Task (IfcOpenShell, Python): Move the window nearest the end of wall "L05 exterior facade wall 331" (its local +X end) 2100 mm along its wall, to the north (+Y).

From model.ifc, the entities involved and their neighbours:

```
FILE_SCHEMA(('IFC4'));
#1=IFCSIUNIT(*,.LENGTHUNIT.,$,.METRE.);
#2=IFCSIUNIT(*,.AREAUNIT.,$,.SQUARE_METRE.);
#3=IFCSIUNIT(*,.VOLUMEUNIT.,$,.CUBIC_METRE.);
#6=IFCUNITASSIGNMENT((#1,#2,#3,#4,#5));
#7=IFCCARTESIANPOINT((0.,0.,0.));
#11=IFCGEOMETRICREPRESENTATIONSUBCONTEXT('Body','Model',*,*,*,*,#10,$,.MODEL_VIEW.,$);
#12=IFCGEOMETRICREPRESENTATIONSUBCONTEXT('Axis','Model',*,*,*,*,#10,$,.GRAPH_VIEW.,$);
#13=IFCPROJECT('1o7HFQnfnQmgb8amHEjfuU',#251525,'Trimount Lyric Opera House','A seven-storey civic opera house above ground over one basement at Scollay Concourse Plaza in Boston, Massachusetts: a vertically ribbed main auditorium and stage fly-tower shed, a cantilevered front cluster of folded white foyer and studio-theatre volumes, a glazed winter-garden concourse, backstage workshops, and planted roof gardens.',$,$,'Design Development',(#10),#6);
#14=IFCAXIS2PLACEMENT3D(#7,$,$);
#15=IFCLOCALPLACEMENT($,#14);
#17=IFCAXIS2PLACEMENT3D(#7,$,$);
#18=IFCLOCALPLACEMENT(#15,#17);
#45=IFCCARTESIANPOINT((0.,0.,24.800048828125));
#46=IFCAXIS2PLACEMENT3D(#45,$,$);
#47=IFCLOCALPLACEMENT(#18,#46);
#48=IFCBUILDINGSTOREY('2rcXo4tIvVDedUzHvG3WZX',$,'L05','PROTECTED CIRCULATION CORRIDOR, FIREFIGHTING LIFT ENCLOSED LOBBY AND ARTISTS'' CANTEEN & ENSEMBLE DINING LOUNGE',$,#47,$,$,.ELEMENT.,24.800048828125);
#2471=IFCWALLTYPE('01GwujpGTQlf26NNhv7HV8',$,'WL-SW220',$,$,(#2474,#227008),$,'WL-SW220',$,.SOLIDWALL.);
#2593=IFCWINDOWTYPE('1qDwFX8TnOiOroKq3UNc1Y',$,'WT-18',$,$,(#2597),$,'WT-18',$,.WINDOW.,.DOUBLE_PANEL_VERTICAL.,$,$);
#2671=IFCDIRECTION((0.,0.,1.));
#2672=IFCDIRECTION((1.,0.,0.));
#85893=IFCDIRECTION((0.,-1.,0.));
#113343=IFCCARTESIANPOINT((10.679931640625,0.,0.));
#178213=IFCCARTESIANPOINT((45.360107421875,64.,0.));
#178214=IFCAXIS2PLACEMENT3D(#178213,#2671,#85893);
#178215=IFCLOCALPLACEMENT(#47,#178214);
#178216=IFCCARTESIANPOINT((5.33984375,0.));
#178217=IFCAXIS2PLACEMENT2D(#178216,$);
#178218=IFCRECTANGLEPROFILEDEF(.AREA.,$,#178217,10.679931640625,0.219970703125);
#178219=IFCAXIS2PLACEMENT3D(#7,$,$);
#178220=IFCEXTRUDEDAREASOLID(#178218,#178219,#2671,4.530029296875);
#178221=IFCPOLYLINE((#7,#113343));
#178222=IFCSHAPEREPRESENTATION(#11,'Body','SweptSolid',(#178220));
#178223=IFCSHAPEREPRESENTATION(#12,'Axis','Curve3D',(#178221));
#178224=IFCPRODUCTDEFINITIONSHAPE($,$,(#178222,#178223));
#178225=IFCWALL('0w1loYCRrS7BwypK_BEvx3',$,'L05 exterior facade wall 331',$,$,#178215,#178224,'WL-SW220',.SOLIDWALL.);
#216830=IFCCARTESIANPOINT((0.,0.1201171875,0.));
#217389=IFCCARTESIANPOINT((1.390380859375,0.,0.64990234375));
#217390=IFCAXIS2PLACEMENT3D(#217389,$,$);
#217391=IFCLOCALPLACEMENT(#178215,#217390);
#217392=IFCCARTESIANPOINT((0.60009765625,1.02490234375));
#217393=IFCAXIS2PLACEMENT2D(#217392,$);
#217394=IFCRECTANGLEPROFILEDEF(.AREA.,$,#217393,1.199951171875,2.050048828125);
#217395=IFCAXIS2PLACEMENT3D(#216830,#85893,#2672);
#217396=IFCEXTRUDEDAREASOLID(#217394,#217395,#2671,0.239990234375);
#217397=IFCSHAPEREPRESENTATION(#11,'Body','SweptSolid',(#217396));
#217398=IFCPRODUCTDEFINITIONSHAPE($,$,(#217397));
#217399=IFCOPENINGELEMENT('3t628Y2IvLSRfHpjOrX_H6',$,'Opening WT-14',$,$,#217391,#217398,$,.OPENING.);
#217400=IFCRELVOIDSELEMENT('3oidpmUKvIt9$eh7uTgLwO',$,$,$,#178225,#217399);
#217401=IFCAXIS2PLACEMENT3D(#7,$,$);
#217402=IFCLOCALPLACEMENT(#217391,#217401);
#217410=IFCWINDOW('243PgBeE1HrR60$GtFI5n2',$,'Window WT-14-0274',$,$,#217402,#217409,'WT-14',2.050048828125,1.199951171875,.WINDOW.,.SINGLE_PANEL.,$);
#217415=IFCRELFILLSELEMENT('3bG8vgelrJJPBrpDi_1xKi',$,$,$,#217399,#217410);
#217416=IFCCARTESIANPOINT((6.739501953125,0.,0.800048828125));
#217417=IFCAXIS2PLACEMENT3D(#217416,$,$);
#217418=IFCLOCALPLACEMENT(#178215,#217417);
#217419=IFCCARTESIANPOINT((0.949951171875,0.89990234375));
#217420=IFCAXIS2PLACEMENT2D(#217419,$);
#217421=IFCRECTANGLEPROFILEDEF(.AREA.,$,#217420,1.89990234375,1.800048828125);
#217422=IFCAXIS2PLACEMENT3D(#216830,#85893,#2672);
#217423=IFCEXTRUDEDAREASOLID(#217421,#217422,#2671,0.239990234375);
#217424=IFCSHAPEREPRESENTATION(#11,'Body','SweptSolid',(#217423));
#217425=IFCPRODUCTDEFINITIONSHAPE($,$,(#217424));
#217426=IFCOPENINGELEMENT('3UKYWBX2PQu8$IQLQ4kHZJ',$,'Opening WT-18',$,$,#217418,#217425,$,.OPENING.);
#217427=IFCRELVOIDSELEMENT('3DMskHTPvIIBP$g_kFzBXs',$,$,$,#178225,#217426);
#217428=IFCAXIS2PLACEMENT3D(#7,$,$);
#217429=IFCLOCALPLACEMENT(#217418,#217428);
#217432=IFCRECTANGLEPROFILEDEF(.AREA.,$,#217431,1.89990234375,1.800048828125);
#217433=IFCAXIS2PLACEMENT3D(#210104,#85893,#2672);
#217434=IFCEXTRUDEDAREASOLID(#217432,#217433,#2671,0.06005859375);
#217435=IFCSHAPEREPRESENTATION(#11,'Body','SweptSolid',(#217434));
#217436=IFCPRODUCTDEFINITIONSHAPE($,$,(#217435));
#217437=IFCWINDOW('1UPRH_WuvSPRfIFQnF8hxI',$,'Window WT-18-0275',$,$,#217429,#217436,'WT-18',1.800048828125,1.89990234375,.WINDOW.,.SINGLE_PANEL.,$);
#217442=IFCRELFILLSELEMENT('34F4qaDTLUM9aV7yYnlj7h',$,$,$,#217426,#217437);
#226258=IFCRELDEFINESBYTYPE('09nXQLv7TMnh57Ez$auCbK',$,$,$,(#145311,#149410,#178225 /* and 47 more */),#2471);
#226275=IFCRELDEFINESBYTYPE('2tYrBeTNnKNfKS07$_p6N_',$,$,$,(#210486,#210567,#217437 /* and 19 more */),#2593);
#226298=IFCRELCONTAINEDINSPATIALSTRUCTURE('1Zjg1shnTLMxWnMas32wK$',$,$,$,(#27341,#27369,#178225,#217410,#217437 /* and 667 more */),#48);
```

```python
import ifcopenshell
import ifcopenshell.api.geometry
import ifcopenshell.util.placement
import ifcopenshell.util.unit

model = ifcopenshell.open("model.ifc")
unit_scale = ifcopenshell.util.unit.calculate_unit_scale(model)

window = model.by_id(217437)
opening = window.FillsVoids[0].RelatingOpeningElement
wall = opening.VoidsElements[0].RelatingBuildingElement

wall_matrix = ifcopenshell.util.placement.get_local_placement(wall.ObjectPlacement)
shift = wall_matrix[:3, 0] * -2.1 / unit_scale
before = ifcopenshell.util.placement.get_local_placement(window.ObjectPlacement)[:3, 3].copy()

# The window is placed relative to its opening, so it follows when the opening moves.
matrix = ifcopenshell.util.placement.get_local_placement(opening.ObjectPlacement)
matrix[:3, 3] += shift
ifcopenshell.api.geometry.edit_object_placement(
    model, product=opening, matrix=matrix, is_si=False, should_transform_children=True
)

after = ifcopenshell.util.placement.get_local_placement(window.ObjectPlacement)[:3, 3]
print("window moved by", (after - before).round(3) + 0.0)

model.write("model_updated.ifc")
```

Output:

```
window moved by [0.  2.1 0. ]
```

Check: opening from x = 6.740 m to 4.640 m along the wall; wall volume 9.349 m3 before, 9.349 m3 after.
